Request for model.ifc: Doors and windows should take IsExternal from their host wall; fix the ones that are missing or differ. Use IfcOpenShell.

First a look at what the model holds.

```python
import ifcopenshell
import ifcopenshell.util.element

model = ifcopenshell.open("model.ifc")
print(model.schema)
seen = {}
for e in model.by_type("IfcDoor") + model.by_type("IfcWindow"):
    if not e.FillsVoids:
        continue
    host = e.FillsVoids[0].RelatingOpeningElement.VoidsElements[0].RelatingBuildingElement
    own = ifcopenshell.util.element.get_pset(e, f"Pset_{e.is_a()[3:].removesuffix('StandardCase')}Common", "IsExternal")
    wall = ifcopenshell.util.element.get_pset(host, "Pset_WallCommon", "IsExternal")
    seen[e.is_a(), own, wall] = seen.get((e.is_a(), own, wall), 0) + 1
for (cls, own, wall), count in sorted(seen.items(), key=str):
    print(count, cls, "IsExternal:", own, "| host wall:", wall)
```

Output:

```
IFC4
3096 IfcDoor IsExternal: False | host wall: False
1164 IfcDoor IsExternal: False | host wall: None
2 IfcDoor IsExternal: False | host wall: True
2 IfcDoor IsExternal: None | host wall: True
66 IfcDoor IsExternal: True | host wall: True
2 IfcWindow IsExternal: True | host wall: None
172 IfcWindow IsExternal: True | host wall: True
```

```python
import ifcopenshell
import ifcopenshell.api.pset
import ifcopenshell.util.element

model = ifcopenshell.open("model.ifc")

count = 0
for ifc_class, pset_name in (("IfcDoor", "Pset_DoorCommon"), ("IfcWindow", "Pset_WindowCommon")):
    for e in model.by_type(ifc_class):
        if not e.FillsVoids:
            continue
        host = e.FillsVoids[0].RelatingOpeningElement.VoidsElements[0].RelatingBuildingElement
        external = ifcopenshell.util.element.get_pset(host, "Pset_WallCommon", "IsExternal")
        if external is None or ifcopenshell.util.element.get_pset(e, pset_name, "IsExternal") == external:
            continue
        found = ifcopenshell.util.element.get_pset(e, pset_name, should_inherit=False)
        if found:
            pset = model.by_id(found["id"])
            if len(ifcopenshell.util.element.get_elements_by_pset(pset)) > 1:
                pset = ifcopenshell.api.pset.unshare_pset(model, products=[e], pset=pset)[0]
        else:
            pset = ifcopenshell.api.pset.add_pset(model, product=e, name=pset_name)
        ifcopenshell.api.pset.edit_pset(model, pset=pset, properties={"IsExternal": external})
        count += 1

print(count, "updated")

model.write("model_v2.ifc")
```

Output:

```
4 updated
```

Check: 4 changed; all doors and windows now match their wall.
